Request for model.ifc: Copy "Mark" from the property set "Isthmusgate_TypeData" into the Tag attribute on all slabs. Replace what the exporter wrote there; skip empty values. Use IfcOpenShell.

First a look at what the model holds.

```python
import ifcopenshell
import ifcopenshell.util.element

model = ifcopenshell.open("model.ifc")
print(model.schema)
slabs = model.by_type("IfcSlab")
print(len(slabs), "slabs")
for e in slabs[:8]:
    source = ifcopenshell.util.element.get_pset(e, "Isthmusgate_TypeData", "Mark")
    target = e.Tag
    print(e.id(), repr(source), repr(target), sep=" | ")
```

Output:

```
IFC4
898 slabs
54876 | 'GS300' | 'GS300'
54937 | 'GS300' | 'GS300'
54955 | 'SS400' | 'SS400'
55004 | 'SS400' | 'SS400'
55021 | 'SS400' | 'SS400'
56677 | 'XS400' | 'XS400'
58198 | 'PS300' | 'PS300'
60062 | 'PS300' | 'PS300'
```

```python
import ifcopenshell
import ifcopenshell.util.element

model = ifcopenshell.open("model.ifc")

count = 0
for e in model.by_type("IfcSlab"):
    value = ifcopenshell.util.element.get_pset(e, "Isthmusgate_TypeData", "Mark")
    current = e.Tag
    if not value or not value.strip() or current == value:
        continue
    e.Tag = value
    count += 1

print(count, "slabs updated")

model.write("model_edited.ifc")
```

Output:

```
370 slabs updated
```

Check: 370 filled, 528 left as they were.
